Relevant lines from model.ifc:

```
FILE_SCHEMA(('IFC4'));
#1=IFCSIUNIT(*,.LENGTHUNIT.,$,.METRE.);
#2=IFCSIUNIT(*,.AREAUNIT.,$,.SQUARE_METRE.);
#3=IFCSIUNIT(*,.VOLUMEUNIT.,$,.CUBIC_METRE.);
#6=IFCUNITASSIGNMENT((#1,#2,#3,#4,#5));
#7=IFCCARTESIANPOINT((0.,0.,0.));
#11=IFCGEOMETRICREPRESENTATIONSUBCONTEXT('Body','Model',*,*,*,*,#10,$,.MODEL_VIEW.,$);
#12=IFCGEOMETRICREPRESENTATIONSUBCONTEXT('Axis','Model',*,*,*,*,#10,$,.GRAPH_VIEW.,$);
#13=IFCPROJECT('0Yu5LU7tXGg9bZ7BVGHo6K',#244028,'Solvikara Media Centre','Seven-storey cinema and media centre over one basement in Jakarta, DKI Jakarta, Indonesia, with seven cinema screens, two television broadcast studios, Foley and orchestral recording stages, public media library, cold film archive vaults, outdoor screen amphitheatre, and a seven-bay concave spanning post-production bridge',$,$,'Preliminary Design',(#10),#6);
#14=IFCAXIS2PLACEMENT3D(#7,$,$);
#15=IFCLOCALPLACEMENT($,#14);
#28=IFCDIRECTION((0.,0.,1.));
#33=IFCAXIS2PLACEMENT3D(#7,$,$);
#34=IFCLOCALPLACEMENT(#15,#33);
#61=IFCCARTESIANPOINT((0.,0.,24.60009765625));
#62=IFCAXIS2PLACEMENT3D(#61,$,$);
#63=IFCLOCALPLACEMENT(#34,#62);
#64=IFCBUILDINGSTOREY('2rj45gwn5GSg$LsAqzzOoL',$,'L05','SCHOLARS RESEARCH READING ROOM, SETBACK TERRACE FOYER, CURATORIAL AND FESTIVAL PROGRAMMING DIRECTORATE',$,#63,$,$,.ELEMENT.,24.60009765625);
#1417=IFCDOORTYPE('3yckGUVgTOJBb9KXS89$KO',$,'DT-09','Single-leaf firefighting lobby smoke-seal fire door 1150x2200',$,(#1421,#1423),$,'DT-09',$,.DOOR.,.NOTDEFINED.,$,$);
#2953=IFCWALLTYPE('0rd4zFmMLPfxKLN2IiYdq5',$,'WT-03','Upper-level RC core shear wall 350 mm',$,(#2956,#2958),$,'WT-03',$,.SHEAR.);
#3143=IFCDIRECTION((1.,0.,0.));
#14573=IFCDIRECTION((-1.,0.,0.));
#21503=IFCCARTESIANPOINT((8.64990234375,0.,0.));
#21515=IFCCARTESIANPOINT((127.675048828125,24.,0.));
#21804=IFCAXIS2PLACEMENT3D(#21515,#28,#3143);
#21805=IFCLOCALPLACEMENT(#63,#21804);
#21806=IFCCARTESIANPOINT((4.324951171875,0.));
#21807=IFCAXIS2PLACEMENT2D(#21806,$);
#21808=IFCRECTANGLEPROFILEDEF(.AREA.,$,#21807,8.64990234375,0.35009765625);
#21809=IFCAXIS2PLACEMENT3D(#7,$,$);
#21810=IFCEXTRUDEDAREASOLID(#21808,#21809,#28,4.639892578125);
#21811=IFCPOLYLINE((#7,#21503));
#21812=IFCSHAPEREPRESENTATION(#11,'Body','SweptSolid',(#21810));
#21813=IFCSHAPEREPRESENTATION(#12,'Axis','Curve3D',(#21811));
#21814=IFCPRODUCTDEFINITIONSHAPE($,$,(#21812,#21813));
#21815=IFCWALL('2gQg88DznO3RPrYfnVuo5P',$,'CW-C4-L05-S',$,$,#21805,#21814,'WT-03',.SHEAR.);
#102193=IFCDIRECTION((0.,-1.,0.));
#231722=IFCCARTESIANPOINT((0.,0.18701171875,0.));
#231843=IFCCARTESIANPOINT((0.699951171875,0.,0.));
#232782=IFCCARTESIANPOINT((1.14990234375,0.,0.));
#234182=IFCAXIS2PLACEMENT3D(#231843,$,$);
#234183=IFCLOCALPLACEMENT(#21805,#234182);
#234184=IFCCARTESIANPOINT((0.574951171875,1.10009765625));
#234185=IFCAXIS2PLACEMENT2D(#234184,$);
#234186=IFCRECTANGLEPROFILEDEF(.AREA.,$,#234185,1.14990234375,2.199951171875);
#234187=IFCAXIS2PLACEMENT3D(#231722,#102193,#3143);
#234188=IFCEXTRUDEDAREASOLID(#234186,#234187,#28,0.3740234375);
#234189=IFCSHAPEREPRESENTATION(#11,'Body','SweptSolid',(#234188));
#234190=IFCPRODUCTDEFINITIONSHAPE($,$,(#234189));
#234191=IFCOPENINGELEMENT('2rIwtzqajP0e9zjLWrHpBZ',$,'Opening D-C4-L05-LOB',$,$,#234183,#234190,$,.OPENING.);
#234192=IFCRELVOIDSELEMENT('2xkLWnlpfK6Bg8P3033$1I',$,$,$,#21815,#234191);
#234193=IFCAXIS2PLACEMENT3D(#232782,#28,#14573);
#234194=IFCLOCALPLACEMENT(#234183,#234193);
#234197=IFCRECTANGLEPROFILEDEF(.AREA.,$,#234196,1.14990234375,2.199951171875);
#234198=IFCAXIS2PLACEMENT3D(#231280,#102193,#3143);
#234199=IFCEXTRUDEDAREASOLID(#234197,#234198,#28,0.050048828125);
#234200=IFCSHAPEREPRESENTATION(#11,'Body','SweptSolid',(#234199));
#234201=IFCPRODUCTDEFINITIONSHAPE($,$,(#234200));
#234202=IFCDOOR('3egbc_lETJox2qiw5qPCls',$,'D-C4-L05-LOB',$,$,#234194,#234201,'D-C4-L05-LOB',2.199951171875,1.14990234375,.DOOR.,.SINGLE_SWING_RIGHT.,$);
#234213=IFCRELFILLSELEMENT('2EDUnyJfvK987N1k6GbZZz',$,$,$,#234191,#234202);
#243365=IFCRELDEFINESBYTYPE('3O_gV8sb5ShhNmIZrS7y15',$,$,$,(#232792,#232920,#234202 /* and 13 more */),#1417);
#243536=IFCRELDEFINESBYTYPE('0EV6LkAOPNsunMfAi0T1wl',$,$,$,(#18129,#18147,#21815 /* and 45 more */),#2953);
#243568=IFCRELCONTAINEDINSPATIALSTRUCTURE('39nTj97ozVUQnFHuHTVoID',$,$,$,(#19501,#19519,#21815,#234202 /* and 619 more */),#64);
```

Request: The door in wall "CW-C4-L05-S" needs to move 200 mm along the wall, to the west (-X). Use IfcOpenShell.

```python
import ifcopenshell
import ifcopenshell.api.geometry
import ifcopenshell.util.placement
import ifcopenshell.util.unit

model = ifcopenshell.open("model.ifc")
unit_scale = ifcopenshell.util.unit.calculate_unit_scale(model)

door = model.by_guid("3egbc_lETJox2qiw5qPCls")
opening = door.FillsVoids[0].RelatingOpeningElement
wall = opening.VoidsElements[0].RelatingBuildingElement

wall_matrix = ifcopenshell.util.placement.get_local_placement(wall.ObjectPlacement)
shift = wall_matrix[:3, 0] * -0.2 / unit_scale
before = ifcopenshell.util.placement.get_local_placement(door.ObjectPlacement)[:3, 3].copy()

# The door is placed relative to its opening, so it follows when the opening moves.
matrix = ifcopenshell.util.placement.get_local_placement(opening.ObjectPlacement)
matrix[:3, 3] += shift
ifcopenshell.api.geometry.edit_object_placement(
    model, product=opening, matrix=matrix, is_si=False, should_transform_children=True
)

after = ifcopenshell.util.placement.get_local_placement(door.ObjectPlacement)[:3, 3]
print("door moved by", (after - before).round(3) + 0.0)

model.write("model_v2.ifc")
```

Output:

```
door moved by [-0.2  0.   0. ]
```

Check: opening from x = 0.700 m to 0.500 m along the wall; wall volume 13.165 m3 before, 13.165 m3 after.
